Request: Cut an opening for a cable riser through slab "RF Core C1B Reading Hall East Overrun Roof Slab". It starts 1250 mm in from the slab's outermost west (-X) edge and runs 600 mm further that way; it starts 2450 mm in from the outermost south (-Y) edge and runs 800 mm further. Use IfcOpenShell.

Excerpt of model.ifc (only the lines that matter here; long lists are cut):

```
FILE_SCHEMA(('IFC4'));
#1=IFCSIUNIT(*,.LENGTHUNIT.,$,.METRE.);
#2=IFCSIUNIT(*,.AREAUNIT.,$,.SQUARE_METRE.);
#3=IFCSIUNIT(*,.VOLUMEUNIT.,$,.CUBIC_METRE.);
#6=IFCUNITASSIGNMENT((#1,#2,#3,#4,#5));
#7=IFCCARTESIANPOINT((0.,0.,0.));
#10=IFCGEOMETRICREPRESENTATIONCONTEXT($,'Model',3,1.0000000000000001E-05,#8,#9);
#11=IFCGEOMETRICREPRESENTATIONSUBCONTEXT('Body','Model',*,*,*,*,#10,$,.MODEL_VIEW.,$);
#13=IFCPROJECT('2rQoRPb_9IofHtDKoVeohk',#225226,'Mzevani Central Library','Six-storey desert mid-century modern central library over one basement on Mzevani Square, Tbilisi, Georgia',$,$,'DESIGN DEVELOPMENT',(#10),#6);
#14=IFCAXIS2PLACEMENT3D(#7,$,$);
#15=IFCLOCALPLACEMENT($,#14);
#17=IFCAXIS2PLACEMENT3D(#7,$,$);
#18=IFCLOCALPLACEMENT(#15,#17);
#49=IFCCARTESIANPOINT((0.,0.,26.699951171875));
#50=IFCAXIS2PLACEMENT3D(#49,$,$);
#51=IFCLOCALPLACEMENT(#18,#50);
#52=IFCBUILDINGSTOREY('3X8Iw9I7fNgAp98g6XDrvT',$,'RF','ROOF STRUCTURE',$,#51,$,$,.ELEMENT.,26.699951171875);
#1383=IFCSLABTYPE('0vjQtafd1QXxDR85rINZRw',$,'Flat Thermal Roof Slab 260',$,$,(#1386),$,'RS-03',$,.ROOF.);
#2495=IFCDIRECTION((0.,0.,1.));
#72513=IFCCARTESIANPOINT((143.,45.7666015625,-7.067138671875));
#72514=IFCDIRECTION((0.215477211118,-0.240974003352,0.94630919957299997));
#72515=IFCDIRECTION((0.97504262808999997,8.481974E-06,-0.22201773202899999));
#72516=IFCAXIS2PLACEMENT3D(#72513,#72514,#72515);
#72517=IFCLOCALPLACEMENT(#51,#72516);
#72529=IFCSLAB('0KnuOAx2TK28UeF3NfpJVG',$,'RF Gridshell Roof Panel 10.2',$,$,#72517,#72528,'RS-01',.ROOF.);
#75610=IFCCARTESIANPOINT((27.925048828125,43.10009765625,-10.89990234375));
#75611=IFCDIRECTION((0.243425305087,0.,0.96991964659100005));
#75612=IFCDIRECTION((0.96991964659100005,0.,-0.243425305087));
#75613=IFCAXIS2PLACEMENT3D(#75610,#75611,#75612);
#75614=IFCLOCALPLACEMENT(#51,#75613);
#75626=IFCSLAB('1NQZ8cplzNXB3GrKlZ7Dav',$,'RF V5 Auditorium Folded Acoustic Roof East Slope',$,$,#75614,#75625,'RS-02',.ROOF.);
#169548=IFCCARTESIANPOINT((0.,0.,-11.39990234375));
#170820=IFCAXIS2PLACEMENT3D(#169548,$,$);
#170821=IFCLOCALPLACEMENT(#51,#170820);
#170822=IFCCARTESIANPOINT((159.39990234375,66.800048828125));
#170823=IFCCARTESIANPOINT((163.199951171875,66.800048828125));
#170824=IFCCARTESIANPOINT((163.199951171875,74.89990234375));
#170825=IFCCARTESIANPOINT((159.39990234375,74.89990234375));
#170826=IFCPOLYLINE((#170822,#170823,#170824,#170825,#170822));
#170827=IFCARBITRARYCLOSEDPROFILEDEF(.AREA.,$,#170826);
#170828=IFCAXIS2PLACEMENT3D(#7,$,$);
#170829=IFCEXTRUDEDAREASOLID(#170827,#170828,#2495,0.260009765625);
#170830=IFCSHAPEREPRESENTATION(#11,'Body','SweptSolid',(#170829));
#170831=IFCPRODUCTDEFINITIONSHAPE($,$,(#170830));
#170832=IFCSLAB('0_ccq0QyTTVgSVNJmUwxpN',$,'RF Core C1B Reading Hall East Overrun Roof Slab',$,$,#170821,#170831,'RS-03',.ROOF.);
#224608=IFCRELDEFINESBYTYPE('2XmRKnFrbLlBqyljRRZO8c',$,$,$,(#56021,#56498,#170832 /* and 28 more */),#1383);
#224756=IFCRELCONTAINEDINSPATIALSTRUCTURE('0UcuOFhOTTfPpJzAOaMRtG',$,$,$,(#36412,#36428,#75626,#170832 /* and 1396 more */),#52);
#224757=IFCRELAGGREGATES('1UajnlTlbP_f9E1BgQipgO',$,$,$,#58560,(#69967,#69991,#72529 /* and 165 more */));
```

```python
import numpy as np
import ifcopenshell
import ifcopenshell.api.feature
import ifcopenshell.api.geometry
import ifcopenshell.api.root
import ifcopenshell.geom
import ifcopenshell.util.placement
import ifcopenshell.util.representation
import ifcopenshell.util.shape
import ifcopenshell.util.unit

model = ifcopenshell.open("model.ifc")
unit_scale = ifcopenshell.util.unit.calculate_unit_scale(model)
settings = ifcopenshell.geom.settings()


def volume(element):
    """Net volume in cubic metres, openings subtracted."""
    shape = ifcopenshell.geom.create_shape(settings, element)
    return ifcopenshell.util.shape.get_volume(shape.geometry)


slab = model.by_id(170832)
before = volume(slab)

# Extent in the slab's own axes, in metres. The edges named are its -X and -Y sides.
slab_shape = ifcopenshell.geom.create_shape(settings, slab)
vertices = ifcopenshell.util.shape.get_vertices(slab_shape.geometry)
x_min, y_min, bottom = vertices.min(axis=0)
top = vertices[:, 2].max()

opening = ifcopenshell.api.root.create_entity(model, ifc_class="IfcOpeningElement", name="Cable riser opening", predefined_type="OPENING")
context = ifcopenshell.util.representation.get_context(model, "Model", "Body", "MODEL_VIEW")
width, depth = 0.6, 0.8
outline = [(0.0, 0.0), (width, 0.0), (width, depth), (0.0, depth), (0.0, 0.0)]
# Overshoot both faces by 50 mm so the cut is clean.
shape = ifcopenshell.api.geometry.add_slab_representation(
    model, context=context, depth=top - bottom + 0.1, polyline=outline
)
ifcopenshell.api.geometry.assign_representation(model, product=opening, representation=shape)

matrix = ifcopenshell.util.placement.get_local_placement(slab.ObjectPlacement)
matrix[:, 3] = matrix @ np.append(np.array([x_min + 1.25, y_min + 2.45, bottom - 0.05]) / unit_scale, 1.0)
ifcopenshell.api.geometry.edit_object_placement(model, product=opening, matrix=matrix, is_si=False)
ifcopenshell.api.feature.add_feature(model, feature=opening, element=slab)

after = volume(slab)

print(f"slab volume {before:.3f} -> {after:.3f} m3")

model.write("model_v2.ifc")
```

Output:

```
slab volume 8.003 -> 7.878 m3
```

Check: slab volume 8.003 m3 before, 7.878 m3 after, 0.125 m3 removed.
